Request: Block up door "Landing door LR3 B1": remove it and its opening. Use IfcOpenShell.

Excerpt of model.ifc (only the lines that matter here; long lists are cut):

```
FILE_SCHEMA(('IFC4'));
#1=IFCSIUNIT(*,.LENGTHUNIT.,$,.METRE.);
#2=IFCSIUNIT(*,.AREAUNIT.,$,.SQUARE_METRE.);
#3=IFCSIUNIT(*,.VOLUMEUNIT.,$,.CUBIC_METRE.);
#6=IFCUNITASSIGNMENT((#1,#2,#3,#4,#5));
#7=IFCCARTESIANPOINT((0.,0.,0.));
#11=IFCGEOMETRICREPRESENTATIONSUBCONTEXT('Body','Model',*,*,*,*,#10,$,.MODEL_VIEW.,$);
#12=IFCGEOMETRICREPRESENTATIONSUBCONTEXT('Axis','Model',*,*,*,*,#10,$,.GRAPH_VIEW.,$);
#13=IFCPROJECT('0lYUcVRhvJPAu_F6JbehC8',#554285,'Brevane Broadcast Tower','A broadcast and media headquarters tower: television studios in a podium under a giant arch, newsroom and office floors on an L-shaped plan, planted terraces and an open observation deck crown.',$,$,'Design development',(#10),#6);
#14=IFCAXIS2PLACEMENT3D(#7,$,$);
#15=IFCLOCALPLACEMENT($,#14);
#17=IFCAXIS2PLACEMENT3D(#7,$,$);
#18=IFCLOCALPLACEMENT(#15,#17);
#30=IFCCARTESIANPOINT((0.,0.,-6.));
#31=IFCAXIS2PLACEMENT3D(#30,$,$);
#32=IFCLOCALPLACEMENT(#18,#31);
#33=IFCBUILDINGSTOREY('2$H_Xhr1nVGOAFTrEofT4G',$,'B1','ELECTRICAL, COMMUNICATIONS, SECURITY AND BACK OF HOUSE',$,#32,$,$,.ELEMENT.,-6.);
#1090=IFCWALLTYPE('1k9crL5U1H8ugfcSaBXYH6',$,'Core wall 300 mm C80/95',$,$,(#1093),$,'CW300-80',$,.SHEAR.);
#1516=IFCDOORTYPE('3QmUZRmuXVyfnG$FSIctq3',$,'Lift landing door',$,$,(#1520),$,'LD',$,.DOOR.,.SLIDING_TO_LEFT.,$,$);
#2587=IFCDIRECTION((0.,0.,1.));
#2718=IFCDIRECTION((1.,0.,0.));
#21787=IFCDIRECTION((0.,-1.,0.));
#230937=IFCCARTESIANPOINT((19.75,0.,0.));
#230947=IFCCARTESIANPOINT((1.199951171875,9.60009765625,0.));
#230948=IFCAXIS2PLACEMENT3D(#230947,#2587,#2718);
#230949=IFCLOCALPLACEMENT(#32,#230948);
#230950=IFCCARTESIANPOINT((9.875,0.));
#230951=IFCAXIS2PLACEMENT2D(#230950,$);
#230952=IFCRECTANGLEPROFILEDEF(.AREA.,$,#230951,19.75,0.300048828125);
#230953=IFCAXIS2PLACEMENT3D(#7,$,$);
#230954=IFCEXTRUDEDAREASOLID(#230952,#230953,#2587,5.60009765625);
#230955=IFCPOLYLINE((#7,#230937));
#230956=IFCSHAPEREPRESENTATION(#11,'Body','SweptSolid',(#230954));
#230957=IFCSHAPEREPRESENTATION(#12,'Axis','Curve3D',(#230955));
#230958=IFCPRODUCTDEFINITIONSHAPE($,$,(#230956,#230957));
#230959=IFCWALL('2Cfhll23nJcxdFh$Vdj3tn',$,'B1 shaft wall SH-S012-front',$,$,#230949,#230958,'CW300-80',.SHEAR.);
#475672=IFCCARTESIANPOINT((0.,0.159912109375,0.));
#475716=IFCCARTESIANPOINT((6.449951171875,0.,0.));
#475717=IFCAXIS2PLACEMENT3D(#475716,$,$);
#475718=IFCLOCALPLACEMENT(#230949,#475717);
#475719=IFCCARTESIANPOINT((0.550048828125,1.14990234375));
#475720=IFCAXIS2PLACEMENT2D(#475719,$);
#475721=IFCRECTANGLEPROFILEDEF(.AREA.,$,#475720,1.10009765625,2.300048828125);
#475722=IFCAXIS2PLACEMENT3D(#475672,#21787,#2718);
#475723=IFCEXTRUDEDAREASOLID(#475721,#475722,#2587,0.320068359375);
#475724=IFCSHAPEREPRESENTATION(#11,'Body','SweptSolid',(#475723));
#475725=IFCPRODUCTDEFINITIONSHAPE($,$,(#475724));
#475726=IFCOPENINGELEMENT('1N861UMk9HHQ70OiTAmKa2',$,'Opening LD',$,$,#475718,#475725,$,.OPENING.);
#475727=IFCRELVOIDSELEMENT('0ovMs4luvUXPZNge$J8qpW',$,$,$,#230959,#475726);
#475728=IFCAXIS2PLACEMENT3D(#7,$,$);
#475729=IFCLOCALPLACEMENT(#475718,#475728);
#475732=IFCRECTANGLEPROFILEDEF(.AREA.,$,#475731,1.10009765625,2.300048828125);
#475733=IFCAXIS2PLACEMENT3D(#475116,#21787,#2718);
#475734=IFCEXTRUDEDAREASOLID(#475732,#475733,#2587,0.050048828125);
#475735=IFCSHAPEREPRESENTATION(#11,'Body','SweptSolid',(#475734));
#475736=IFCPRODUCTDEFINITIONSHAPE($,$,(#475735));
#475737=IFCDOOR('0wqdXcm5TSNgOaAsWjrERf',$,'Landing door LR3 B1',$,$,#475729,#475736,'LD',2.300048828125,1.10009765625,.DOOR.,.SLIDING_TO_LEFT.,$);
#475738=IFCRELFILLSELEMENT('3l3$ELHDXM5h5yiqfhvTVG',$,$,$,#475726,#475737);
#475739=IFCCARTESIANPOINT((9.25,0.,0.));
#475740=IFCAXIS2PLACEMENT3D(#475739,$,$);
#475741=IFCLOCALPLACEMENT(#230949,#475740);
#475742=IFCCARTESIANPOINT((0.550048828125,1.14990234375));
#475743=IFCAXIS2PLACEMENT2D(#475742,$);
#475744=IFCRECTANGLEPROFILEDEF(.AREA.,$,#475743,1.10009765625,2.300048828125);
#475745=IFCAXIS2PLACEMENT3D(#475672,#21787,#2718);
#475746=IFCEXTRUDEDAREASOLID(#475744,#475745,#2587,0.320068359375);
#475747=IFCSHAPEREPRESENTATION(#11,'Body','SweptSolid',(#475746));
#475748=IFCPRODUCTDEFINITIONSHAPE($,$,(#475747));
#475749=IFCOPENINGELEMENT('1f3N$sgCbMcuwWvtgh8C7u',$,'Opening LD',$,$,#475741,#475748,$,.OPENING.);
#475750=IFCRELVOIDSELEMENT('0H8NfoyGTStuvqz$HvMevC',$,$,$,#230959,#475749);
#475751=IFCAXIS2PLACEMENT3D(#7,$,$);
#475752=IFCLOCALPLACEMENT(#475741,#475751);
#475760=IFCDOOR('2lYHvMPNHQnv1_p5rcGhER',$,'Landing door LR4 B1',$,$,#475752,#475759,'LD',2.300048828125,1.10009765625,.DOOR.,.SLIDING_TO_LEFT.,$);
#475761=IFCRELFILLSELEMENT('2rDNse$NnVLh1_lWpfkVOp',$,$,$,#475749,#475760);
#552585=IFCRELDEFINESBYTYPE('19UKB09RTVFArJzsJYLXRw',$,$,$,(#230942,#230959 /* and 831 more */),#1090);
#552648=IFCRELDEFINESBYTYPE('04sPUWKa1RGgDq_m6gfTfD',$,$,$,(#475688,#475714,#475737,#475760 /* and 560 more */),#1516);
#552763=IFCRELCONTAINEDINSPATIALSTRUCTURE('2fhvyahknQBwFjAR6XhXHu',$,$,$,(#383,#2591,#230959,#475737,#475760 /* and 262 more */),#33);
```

```python
import ifcopenshell
import ifcopenshell.api.feature
import ifcopenshell.api.root
import ifcopenshell.geom
import ifcopenshell.util.shape

model = ifcopenshell.open("model.ifc")
settings = ifcopenshell.geom.settings()


def volume(element):
    """Net volume in cubic metres, openings subtracted."""
    shape = ifcopenshell.geom.create_shape(settings, element)
    return ifcopenshell.util.shape.get_volume(shape.geometry)


door = model.by_id(475737)
opening = door.FillsVoids[0].RelatingOpeningElement
wall = opening.VoidsElements[0].RelatingBuildingElement
before = volume(wall)

ifcopenshell.api.root.remove_product(model, product=door)
ifcopenshell.api.feature.remove_feature(model, feature=opening)

after = volume(wall)

print(f"wall volume {before:.3f} -> {after:.3f} m3")

model.write("model_updated.ifc")
```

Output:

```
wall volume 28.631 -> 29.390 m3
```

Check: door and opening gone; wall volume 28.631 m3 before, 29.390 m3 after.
